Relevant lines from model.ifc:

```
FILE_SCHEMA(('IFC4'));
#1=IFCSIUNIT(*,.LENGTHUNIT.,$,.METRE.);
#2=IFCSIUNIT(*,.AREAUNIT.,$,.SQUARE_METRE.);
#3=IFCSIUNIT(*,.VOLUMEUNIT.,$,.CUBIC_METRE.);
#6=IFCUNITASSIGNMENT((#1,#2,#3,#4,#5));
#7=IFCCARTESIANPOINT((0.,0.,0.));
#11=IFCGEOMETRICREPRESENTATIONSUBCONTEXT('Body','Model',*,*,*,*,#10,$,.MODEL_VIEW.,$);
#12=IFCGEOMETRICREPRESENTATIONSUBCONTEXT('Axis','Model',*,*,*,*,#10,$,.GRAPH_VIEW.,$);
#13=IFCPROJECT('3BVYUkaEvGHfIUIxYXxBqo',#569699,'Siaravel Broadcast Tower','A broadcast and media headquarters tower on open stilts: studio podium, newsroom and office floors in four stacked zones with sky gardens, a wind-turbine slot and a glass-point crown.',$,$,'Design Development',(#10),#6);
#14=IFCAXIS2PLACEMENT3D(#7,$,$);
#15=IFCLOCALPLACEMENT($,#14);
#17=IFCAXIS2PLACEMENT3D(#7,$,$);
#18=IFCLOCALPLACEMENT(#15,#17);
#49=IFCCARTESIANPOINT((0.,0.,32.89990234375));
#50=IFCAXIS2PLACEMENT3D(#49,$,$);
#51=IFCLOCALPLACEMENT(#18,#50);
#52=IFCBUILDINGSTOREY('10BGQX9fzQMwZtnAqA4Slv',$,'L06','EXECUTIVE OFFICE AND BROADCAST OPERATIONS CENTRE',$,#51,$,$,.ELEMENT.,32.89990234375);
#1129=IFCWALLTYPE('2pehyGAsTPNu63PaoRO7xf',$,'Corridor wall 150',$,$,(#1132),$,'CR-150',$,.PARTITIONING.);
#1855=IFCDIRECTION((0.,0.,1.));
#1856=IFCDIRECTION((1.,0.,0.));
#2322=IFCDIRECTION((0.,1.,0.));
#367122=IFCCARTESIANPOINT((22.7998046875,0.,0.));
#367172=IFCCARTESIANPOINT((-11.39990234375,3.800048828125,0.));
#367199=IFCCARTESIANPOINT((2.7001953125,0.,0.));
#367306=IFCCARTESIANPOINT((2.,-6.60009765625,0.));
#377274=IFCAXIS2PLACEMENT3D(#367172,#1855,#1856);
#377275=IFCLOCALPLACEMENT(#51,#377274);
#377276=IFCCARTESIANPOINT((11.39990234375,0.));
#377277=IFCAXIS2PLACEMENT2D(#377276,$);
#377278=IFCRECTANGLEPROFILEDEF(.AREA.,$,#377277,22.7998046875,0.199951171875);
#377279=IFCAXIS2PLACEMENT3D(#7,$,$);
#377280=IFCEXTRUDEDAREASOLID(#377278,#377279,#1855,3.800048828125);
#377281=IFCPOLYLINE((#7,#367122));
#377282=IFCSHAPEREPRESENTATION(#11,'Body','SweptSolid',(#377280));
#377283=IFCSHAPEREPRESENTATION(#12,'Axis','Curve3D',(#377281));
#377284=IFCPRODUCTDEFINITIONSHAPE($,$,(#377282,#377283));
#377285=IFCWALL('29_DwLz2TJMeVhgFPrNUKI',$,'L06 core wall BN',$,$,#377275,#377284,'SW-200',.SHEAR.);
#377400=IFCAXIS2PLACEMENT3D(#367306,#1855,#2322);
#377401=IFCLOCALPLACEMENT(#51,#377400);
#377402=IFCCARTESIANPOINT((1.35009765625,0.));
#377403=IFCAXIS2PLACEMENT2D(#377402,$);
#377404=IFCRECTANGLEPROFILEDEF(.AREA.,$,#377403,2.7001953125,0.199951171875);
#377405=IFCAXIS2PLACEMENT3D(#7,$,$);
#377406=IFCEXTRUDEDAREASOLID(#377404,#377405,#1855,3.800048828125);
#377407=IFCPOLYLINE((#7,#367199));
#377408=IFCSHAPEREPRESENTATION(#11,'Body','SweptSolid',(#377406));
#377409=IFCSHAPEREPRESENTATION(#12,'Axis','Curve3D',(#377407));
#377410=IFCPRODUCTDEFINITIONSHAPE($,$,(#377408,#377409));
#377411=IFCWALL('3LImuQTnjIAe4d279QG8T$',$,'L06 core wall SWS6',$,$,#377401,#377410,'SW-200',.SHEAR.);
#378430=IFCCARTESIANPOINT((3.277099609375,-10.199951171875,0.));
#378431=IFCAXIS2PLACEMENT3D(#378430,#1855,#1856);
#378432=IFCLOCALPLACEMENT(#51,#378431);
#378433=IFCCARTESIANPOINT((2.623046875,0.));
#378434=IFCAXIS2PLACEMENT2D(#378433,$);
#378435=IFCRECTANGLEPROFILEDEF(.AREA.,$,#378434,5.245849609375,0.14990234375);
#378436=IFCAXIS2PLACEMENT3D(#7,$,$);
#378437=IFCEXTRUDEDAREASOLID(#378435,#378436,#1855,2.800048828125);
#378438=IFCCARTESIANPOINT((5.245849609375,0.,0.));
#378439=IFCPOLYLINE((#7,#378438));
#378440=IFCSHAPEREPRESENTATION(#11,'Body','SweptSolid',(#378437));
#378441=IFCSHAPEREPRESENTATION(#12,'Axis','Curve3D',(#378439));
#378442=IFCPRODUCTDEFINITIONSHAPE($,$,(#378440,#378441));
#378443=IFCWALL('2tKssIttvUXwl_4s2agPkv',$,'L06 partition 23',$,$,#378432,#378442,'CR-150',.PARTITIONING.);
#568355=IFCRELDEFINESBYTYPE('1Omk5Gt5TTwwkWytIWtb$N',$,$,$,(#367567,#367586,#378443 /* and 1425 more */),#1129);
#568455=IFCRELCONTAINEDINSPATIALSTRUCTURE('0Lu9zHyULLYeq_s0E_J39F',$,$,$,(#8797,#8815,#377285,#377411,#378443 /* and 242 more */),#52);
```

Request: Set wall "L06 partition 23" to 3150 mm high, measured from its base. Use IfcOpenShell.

```python
import ifcopenshell
import ifcopenshell.geom
import ifcopenshell.util.representation
import ifcopenshell.util.shape
import ifcopenshell.util.unit

model = ifcopenshell.open("model.ifc")
unit_scale = ifcopenshell.util.unit.calculate_unit_scale(model)
settings = ifcopenshell.geom.settings()


def volume(element):
    """Net volume in cubic metres, openings subtracted."""
    shape = ifcopenshell.geom.create_shape(settings, element)
    return ifcopenshell.util.shape.get_volume(shape.geometry)


wall = model.by_guid("2tKssIttvUXwl_4s2agPkv")
before = volume(wall)

body = ifcopenshell.util.representation.get_representation(wall, "Model", "Body")
solid = body.Items[0]
old_height = solid.Depth
solid.Depth = 3.15 / unit_scale
after = volume(wall)

print(f"height {old_height:g} -> {solid.Depth:g}, volume {before:.3f} -> {after:.3f} m3")

model.write("model-out.ifc")
```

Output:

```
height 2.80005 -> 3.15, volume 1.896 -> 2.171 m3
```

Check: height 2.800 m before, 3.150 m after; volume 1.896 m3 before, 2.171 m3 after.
